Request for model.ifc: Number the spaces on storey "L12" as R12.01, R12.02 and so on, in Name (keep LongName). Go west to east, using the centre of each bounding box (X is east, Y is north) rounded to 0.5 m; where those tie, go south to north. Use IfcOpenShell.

First a look at what the model holds.

```python
import ifcopenshell
import ifcopenshell.util.element
import ifcopenshell.util.placement

model = ifcopenshell.open("model.ifc")
print(model.schema)
storey = next(s for s in model.by_type("IfcBuildingStorey") if s.Name == "L12")
spaces = [e for e in ifcopenshell.util.element.get_decomposition(storey) if e.is_a("IfcSpace")]
for e in sorted(spaces, key=lambda e: e.id()):
    origin = ifcopenshell.util.placement.get_local_placement(e.ObjectPlacement)[:3, 3]
    print(e.id(), e.Name, e.LongName, origin.round(2) + 0.0, sep=" | ")
```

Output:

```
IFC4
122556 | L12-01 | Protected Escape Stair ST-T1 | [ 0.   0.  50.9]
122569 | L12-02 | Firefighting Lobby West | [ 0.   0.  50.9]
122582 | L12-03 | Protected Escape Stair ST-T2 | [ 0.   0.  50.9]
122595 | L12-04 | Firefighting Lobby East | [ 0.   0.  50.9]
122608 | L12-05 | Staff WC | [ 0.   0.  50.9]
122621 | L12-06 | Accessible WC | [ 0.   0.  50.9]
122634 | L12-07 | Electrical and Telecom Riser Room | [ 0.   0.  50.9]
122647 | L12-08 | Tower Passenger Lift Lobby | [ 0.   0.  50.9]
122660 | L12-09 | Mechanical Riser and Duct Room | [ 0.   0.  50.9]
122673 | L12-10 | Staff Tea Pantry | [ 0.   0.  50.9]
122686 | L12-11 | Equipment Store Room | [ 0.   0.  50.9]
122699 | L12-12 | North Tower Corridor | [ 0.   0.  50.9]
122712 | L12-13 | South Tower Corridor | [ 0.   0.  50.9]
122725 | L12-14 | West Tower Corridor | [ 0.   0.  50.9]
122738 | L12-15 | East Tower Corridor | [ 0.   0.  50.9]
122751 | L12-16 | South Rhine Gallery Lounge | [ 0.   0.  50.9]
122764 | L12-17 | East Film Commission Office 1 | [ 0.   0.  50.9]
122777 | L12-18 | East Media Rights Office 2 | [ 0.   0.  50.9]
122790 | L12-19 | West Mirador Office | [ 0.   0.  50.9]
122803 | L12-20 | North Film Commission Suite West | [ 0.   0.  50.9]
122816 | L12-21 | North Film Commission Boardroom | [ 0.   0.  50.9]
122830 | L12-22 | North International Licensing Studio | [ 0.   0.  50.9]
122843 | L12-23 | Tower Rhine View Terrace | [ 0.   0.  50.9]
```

```python
import ifcopenshell
import ifcopenshell.geom
import ifcopenshell.util.element
import ifcopenshell.util.shape

model = ifcopenshell.open("model.ifc")
settings = ifcopenshell.geom.settings()
settings.set("use-world-coords", True)


def centre(element):
    shape = ifcopenshell.geom.create_shape(settings, element)
    return ifcopenshell.util.shape.get_bbox_centroid(shape.geometry)


storey = next(s for s in model.by_type("IfcBuildingStorey") if s.Name == "L12")
spaces = [e for e in ifcopenshell.util.element.get_decomposition(storey) if e.is_a("IfcSpace")]

# Insertion points can sit at a corner or the storey origin, so sort by the geometry (in metres).
centres = {e: centre(e) for e in spaces}
spaces.sort(key=lambda e: (round(centres[e][0] / 0.5), centres[e][1]))

for i, e in enumerate(spaces, start=1):
    number = f"R12.{i:02d}"
    e.Name = number
    print(e.id(), number)

model.write("model_rev.ifc")
```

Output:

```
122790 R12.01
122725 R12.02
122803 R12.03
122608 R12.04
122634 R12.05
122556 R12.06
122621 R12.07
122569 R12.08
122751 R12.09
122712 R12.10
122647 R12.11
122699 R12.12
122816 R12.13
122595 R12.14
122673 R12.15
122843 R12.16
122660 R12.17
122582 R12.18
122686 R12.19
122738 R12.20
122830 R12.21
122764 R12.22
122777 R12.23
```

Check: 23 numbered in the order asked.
